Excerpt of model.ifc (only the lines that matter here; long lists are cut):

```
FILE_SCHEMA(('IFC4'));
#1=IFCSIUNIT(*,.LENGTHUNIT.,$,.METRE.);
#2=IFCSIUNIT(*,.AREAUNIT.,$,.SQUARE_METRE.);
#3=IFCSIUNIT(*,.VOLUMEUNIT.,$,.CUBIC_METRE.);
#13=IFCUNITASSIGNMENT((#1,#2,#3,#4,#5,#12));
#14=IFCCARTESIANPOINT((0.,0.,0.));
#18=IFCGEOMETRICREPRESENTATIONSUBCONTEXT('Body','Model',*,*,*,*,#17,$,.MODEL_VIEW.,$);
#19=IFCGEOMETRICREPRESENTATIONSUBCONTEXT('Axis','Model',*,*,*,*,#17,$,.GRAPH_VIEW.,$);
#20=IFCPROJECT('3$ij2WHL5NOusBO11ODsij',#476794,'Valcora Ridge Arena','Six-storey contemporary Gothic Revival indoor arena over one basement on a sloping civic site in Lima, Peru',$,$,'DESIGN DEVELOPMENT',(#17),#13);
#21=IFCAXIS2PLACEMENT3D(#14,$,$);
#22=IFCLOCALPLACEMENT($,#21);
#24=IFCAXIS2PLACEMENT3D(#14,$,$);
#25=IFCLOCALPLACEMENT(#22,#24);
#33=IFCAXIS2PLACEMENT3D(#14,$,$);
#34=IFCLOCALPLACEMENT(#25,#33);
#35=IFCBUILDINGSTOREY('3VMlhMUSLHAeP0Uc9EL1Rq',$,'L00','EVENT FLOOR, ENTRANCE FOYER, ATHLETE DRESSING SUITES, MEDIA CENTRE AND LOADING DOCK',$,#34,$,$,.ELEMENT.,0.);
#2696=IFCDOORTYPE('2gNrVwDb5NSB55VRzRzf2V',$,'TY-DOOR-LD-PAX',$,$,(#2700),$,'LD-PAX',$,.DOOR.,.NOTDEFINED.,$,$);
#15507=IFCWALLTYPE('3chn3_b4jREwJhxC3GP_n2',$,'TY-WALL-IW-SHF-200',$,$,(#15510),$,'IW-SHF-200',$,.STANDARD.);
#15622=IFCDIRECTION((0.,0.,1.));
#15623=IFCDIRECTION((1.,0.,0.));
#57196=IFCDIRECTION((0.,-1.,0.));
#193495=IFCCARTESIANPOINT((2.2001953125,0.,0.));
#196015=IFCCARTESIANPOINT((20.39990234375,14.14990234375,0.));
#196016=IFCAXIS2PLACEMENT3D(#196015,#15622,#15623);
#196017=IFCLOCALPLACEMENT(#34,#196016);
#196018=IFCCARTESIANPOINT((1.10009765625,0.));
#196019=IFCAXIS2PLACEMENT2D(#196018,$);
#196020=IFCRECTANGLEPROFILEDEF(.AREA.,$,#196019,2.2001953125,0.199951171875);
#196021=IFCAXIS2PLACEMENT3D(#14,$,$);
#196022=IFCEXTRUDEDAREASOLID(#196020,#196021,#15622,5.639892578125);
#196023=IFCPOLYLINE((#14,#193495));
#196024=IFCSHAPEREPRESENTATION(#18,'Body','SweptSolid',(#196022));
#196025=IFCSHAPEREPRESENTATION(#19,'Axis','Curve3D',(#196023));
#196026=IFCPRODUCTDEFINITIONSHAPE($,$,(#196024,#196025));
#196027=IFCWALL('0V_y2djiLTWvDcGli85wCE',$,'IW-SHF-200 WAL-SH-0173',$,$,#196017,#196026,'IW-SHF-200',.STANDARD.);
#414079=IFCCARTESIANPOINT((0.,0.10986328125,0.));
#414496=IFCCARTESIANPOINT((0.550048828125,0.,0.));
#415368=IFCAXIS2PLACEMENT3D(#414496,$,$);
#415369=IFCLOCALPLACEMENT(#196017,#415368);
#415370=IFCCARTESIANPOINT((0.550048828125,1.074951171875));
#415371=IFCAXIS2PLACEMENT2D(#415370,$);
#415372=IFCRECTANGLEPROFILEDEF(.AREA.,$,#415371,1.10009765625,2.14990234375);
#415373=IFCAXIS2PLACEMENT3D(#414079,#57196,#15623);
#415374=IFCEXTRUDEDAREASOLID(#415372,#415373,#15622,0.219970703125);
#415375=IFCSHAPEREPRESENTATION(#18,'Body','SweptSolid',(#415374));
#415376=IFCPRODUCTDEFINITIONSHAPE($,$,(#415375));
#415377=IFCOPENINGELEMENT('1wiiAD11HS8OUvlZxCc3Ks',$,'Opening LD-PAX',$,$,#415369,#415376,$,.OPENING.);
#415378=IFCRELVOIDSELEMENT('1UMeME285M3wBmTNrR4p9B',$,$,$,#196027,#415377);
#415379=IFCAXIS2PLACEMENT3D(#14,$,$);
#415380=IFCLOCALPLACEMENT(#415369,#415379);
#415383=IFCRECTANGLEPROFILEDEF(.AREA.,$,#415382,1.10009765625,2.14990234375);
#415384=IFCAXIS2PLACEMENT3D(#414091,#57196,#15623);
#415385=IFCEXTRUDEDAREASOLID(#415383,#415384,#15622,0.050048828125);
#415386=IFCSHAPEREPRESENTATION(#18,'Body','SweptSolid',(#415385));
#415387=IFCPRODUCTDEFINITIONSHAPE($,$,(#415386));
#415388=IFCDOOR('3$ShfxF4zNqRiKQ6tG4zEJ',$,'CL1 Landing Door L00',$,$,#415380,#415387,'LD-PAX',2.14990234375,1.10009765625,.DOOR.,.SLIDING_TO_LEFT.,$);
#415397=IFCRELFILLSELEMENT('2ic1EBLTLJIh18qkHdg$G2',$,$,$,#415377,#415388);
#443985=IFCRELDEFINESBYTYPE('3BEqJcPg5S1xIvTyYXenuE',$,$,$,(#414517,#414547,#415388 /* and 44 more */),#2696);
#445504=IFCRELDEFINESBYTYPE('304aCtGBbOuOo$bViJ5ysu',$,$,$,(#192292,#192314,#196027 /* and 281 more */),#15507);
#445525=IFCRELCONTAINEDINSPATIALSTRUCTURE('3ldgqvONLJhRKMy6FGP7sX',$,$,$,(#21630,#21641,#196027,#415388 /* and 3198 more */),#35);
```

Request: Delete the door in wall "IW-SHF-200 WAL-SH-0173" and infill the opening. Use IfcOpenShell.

```python
import ifcopenshell
import ifcopenshell.api.feature
import ifcopenshell.api.root
import ifcopenshell.geom
import ifcopenshell.util.shape

model = ifcopenshell.open("model.ifc")
settings = ifcopenshell.geom.settings()


def volume(element):
    """Net volume in cubic metres, openings subtracted."""
    shape = ifcopenshell.geom.create_shape(settings, element)
    return ifcopenshell.util.shape.get_volume(shape.geometry)


door = model.by_id(415388)
opening = door.FillsVoids[0].RelatingOpeningElement
wall = opening.VoidsElements[0].RelatingBuildingElement
before = volume(wall)

ifcopenshell.api.root.remove_product(model, product=door)
ifcopenshell.api.feature.remove_feature(model, feature=opening)

after = volume(wall)

print(f"wall volume {before:.3f} -> {after:.3f} m3")

model.write("model-out.ifc")
```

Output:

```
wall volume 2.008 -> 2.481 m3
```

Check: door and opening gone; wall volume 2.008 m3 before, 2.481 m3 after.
